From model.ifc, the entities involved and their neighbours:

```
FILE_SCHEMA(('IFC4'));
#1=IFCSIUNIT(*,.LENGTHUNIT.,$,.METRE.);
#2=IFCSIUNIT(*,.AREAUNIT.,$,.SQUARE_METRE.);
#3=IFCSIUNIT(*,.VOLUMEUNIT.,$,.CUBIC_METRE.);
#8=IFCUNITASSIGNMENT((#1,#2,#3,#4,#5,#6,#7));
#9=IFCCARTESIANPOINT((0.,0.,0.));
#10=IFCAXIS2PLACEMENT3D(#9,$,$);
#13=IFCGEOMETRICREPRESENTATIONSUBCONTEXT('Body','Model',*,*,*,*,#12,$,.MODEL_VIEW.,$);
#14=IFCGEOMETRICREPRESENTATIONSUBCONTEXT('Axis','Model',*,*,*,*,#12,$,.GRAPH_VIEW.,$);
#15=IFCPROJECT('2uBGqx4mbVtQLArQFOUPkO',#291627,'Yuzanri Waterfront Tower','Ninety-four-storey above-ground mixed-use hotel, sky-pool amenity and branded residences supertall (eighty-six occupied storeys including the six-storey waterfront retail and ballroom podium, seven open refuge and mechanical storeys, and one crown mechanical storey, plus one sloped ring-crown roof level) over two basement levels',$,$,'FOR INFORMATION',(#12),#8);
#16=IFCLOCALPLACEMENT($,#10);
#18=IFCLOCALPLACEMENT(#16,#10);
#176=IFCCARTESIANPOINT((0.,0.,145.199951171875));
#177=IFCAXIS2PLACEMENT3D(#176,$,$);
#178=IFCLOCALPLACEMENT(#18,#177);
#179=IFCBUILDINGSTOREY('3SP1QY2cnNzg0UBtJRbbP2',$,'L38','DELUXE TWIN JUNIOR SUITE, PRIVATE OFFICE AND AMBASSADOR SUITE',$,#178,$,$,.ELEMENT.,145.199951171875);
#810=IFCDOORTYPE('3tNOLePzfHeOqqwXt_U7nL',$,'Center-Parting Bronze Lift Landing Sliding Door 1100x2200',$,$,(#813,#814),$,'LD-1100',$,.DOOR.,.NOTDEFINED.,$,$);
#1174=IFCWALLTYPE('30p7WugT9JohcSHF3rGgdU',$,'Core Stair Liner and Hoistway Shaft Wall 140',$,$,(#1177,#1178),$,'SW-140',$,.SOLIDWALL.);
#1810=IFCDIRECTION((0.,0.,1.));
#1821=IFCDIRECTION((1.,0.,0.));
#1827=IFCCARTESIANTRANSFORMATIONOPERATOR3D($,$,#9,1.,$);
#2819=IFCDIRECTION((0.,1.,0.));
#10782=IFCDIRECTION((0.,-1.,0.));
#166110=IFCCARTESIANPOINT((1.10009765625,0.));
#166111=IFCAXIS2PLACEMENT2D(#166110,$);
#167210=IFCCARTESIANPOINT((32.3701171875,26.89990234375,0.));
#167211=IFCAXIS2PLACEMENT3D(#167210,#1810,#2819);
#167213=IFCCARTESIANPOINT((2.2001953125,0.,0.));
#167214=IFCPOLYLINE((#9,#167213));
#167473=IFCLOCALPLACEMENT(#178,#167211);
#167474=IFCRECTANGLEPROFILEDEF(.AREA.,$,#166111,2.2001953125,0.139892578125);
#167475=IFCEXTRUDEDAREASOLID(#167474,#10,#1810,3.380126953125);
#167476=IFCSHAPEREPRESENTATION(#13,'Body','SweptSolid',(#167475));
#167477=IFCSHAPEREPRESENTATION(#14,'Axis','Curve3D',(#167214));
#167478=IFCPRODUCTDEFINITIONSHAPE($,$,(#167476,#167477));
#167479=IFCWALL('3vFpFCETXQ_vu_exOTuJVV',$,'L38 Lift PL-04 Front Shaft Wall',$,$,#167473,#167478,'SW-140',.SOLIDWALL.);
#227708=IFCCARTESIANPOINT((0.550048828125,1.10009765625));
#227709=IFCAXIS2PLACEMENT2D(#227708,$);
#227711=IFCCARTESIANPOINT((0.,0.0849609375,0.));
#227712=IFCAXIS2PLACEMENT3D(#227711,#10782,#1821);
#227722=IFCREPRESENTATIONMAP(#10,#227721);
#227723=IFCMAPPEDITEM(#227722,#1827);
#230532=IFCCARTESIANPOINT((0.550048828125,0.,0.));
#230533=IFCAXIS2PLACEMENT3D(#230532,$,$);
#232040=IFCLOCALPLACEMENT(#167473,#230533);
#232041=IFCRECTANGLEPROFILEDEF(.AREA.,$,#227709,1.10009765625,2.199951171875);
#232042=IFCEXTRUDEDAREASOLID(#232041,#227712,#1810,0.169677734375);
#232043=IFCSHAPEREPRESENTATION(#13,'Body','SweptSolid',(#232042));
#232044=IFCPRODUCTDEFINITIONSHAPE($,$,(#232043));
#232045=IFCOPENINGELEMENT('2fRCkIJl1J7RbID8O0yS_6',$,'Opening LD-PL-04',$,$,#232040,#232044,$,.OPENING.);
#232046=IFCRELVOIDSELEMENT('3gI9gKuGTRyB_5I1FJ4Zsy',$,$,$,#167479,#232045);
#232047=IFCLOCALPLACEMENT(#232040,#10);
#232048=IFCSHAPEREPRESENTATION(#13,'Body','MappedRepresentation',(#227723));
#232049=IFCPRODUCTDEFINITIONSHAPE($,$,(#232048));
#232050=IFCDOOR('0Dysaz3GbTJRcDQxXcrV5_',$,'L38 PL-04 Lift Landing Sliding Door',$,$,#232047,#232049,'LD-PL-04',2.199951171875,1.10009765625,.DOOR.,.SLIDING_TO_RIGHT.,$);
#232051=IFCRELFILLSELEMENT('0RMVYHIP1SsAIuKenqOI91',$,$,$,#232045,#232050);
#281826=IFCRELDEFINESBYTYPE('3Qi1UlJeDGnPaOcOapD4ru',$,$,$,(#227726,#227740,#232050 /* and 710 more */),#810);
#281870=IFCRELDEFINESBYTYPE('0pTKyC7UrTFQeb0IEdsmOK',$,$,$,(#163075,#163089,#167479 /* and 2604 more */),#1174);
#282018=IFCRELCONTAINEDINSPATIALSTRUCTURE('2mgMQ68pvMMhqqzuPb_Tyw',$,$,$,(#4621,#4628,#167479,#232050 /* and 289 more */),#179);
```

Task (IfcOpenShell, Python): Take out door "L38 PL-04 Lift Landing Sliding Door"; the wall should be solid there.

```python
import ifcopenshell
import ifcopenshell.api.feature
import ifcopenshell.api.root
import ifcopenshell.geom
import ifcopenshell.util.shape

model = ifcopenshell.open("model.ifc")
settings = ifcopenshell.geom.settings()


def volume(element):
    """Net volume in cubic metres, openings subtracted."""
    shape = ifcopenshell.geom.create_shape(settings, element)
    return ifcopenshell.util.shape.get_volume(shape.geometry)


door = model.by_guid("0Dysaz3GbTJRcDQxXcrV5_")
opening = door.FillsVoids[0].RelatingOpeningElement
wall = opening.VoidsElements[0].RelatingBuildingElement
before = volume(wall)

ifcopenshell.api.root.remove_product(model, product=door)
ifcopenshell.api.feature.remove_feature(model, feature=opening)

after = volume(wall)

print(f"wall volume {before:.3f} -> {after:.3f} m3")

model.write("model-out.ifc")
```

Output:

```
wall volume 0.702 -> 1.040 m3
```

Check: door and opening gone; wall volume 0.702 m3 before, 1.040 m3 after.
